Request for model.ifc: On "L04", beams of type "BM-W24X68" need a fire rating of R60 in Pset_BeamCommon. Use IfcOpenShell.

First a look at what the model holds.

```python
import ifcopenshell
import ifcopenshell.util.element

model = ifcopenshell.open("model.ifc")
print(model.schema)
storey = next(s for s in model.by_type("IfcBuildingStorey") if s.Name == "L04")
beams = [e for e in ifcopenshell.util.element.get_decomposition(storey) if e.is_a("IfcBeam")]
seen = {}
for e in beams:
    element_type = ifcopenshell.util.element.get_type(e)
    key = (element_type.Name if element_type != e and element_type else None, ifcopenshell.util.element.get_pset(e, "Pset_BeamCommon", "FireRating"))
    seen[key] = seen.get(key, 0) + 1
for (name, value), count in sorted(seen.items(), key=str):
    print(count, "x", name, "|", value)
```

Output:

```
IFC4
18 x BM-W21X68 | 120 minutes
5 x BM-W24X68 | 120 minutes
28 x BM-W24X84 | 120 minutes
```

```python
import ifcopenshell
import ifcopenshell.api.pset
import ifcopenshell.util.element

model = ifcopenshell.open("model.ifc")

storey = next(s for s in model.by_type("IfcBuildingStorey") if s.Name == "L04")
beams = [e for e in ifcopenshell.util.element.get_decomposition(storey) if e.is_a("IfcBeam")]

count = 0
for e in beams:
    element_type = ifcopenshell.util.element.get_type(e)
    if element_type in (None, e) or element_type.Name != "BM-W24X68":
        continue
    # add_pset returns the element's existing set when there is one.
    pset = ifcopenshell.api.pset.add_pset(model, product=e, name="Pset_BeamCommon")
    ifcopenshell.api.pset.edit_pset(model, pset=pset, properties={"FireRating": "R60"})
    count += 1

print(count, "beams updated")

model.write("model_v2.ifc")
```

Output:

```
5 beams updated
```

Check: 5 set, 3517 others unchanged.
